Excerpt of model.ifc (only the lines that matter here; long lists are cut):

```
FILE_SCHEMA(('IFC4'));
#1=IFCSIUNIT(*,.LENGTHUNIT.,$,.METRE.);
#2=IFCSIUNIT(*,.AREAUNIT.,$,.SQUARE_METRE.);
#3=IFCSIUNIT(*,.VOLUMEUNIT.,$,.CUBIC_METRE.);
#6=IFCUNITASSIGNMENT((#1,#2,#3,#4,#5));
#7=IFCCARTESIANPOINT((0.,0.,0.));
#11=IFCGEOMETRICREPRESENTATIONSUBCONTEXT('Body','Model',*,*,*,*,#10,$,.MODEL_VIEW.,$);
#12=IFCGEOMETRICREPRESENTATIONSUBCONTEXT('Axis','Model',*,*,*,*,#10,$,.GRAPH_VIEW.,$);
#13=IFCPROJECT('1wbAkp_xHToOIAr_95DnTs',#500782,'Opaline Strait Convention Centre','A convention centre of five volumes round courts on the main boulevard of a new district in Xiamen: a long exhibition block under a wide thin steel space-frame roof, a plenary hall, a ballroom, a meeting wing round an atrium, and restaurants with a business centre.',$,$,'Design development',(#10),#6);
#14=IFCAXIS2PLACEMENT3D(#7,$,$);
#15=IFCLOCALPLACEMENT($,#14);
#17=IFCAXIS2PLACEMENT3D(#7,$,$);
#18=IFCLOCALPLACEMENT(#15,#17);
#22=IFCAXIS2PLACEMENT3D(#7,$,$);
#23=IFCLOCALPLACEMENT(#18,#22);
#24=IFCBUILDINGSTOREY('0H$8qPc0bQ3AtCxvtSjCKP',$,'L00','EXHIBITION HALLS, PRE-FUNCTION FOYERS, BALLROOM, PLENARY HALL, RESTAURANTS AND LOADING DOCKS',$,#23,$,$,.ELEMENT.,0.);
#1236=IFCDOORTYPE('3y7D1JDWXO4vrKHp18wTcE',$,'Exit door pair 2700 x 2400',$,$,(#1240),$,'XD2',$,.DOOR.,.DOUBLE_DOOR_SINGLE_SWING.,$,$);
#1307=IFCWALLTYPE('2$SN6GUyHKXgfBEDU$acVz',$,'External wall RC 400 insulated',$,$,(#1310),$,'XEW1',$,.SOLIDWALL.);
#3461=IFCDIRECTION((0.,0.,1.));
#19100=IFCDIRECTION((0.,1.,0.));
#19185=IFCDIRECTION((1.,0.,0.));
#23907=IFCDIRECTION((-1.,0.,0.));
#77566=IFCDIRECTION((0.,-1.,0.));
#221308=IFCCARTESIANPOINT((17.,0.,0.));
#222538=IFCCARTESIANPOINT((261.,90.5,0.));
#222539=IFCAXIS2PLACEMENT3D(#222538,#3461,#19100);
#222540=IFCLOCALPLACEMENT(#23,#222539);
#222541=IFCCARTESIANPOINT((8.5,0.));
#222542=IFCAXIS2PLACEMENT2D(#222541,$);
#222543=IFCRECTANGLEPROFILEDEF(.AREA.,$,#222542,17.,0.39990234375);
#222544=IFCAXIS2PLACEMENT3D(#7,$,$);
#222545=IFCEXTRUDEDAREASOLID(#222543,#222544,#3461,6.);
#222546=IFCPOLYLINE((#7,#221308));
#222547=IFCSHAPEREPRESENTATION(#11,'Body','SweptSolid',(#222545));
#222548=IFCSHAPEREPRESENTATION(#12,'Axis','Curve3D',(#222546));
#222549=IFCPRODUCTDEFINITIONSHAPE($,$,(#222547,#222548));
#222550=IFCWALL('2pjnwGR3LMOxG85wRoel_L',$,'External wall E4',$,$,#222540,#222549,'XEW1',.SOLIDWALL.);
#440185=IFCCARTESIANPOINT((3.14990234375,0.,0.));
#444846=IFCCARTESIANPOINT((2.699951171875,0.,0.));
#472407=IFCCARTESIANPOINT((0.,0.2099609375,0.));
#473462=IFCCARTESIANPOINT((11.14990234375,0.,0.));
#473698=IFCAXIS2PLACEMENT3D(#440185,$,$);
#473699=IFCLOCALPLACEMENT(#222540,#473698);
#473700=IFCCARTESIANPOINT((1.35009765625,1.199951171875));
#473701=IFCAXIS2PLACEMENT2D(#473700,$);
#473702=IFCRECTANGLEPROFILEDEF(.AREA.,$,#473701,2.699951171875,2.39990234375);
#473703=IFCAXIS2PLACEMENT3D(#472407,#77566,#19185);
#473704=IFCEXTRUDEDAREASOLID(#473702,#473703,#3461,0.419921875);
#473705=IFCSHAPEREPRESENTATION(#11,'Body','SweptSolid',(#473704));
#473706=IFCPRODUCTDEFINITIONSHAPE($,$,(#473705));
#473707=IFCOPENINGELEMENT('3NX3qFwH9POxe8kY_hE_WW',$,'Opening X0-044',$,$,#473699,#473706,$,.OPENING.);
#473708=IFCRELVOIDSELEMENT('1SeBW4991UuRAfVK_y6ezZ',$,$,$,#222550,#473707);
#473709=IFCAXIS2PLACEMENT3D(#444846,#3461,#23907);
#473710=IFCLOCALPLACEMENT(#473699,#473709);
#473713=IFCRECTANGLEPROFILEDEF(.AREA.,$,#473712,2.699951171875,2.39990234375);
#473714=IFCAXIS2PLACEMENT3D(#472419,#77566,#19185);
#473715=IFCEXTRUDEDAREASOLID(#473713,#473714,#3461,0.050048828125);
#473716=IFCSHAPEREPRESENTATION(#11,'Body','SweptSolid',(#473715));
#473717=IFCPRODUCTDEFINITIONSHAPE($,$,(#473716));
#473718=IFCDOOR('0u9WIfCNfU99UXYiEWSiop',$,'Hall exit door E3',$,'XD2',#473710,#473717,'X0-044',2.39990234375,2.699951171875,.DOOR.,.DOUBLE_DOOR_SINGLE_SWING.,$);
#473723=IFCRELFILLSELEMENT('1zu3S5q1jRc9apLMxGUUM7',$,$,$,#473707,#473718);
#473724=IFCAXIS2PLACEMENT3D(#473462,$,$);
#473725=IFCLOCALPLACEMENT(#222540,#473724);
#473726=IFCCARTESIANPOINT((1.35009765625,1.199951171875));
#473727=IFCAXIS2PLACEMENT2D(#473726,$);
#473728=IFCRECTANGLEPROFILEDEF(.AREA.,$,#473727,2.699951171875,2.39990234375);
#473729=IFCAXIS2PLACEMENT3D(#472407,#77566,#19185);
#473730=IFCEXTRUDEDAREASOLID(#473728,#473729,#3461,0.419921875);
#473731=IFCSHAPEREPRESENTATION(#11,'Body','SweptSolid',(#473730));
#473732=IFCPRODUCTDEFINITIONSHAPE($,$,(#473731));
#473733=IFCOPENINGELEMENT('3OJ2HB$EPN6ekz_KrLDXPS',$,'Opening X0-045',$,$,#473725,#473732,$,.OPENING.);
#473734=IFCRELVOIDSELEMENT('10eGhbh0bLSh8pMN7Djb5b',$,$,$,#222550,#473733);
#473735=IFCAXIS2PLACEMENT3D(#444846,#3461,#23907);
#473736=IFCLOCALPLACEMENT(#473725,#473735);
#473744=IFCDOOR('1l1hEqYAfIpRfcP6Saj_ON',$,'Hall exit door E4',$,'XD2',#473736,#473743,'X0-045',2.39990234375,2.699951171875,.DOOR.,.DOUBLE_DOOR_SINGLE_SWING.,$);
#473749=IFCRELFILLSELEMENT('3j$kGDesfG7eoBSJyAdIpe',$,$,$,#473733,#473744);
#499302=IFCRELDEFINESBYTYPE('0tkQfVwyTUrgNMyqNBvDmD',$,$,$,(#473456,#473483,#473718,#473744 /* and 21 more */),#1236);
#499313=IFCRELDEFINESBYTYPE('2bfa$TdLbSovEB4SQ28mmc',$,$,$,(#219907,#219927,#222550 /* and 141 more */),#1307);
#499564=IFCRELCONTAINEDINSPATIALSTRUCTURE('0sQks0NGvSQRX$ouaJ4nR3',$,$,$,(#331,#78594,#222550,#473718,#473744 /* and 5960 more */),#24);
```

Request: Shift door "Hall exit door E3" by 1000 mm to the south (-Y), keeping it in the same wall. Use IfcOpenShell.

```python
import ifcopenshell
import ifcopenshell.api.geometry
import ifcopenshell.util.placement
import ifcopenshell.util.unit

model = ifcopenshell.open("model.ifc")
unit_scale = ifcopenshell.util.unit.calculate_unit_scale(model)

door = model.by_guid("0u9WIfCNfU99UXYiEWSiop")
opening = door.FillsVoids[0].RelatingOpeningElement
wall = opening.VoidsElements[0].RelatingBuildingElement

wall_matrix = ifcopenshell.util.placement.get_local_placement(wall.ObjectPlacement)
shift = wall_matrix[:3, 0] * -1 / unit_scale
before = ifcopenshell.util.placement.get_local_placement(door.ObjectPlacement)[:3, 3].copy()

# The door is placed relative to its opening, so it follows when the opening moves.
matrix = ifcopenshell.util.placement.get_local_placement(opening.ObjectPlacement)
matrix[:3, 3] += shift
ifcopenshell.api.geometry.edit_object_placement(
    model, product=opening, matrix=matrix, is_si=False, should_transform_children=True
)

after = ifcopenshell.util.placement.get_local_placement(door.ObjectPlacement)[:3, 3]
print("door moved by", (after - before).round(3) + 0.0)

model.write("model_rev.ifc")
```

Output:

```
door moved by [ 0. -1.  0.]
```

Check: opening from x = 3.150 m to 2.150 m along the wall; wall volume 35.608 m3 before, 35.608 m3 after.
